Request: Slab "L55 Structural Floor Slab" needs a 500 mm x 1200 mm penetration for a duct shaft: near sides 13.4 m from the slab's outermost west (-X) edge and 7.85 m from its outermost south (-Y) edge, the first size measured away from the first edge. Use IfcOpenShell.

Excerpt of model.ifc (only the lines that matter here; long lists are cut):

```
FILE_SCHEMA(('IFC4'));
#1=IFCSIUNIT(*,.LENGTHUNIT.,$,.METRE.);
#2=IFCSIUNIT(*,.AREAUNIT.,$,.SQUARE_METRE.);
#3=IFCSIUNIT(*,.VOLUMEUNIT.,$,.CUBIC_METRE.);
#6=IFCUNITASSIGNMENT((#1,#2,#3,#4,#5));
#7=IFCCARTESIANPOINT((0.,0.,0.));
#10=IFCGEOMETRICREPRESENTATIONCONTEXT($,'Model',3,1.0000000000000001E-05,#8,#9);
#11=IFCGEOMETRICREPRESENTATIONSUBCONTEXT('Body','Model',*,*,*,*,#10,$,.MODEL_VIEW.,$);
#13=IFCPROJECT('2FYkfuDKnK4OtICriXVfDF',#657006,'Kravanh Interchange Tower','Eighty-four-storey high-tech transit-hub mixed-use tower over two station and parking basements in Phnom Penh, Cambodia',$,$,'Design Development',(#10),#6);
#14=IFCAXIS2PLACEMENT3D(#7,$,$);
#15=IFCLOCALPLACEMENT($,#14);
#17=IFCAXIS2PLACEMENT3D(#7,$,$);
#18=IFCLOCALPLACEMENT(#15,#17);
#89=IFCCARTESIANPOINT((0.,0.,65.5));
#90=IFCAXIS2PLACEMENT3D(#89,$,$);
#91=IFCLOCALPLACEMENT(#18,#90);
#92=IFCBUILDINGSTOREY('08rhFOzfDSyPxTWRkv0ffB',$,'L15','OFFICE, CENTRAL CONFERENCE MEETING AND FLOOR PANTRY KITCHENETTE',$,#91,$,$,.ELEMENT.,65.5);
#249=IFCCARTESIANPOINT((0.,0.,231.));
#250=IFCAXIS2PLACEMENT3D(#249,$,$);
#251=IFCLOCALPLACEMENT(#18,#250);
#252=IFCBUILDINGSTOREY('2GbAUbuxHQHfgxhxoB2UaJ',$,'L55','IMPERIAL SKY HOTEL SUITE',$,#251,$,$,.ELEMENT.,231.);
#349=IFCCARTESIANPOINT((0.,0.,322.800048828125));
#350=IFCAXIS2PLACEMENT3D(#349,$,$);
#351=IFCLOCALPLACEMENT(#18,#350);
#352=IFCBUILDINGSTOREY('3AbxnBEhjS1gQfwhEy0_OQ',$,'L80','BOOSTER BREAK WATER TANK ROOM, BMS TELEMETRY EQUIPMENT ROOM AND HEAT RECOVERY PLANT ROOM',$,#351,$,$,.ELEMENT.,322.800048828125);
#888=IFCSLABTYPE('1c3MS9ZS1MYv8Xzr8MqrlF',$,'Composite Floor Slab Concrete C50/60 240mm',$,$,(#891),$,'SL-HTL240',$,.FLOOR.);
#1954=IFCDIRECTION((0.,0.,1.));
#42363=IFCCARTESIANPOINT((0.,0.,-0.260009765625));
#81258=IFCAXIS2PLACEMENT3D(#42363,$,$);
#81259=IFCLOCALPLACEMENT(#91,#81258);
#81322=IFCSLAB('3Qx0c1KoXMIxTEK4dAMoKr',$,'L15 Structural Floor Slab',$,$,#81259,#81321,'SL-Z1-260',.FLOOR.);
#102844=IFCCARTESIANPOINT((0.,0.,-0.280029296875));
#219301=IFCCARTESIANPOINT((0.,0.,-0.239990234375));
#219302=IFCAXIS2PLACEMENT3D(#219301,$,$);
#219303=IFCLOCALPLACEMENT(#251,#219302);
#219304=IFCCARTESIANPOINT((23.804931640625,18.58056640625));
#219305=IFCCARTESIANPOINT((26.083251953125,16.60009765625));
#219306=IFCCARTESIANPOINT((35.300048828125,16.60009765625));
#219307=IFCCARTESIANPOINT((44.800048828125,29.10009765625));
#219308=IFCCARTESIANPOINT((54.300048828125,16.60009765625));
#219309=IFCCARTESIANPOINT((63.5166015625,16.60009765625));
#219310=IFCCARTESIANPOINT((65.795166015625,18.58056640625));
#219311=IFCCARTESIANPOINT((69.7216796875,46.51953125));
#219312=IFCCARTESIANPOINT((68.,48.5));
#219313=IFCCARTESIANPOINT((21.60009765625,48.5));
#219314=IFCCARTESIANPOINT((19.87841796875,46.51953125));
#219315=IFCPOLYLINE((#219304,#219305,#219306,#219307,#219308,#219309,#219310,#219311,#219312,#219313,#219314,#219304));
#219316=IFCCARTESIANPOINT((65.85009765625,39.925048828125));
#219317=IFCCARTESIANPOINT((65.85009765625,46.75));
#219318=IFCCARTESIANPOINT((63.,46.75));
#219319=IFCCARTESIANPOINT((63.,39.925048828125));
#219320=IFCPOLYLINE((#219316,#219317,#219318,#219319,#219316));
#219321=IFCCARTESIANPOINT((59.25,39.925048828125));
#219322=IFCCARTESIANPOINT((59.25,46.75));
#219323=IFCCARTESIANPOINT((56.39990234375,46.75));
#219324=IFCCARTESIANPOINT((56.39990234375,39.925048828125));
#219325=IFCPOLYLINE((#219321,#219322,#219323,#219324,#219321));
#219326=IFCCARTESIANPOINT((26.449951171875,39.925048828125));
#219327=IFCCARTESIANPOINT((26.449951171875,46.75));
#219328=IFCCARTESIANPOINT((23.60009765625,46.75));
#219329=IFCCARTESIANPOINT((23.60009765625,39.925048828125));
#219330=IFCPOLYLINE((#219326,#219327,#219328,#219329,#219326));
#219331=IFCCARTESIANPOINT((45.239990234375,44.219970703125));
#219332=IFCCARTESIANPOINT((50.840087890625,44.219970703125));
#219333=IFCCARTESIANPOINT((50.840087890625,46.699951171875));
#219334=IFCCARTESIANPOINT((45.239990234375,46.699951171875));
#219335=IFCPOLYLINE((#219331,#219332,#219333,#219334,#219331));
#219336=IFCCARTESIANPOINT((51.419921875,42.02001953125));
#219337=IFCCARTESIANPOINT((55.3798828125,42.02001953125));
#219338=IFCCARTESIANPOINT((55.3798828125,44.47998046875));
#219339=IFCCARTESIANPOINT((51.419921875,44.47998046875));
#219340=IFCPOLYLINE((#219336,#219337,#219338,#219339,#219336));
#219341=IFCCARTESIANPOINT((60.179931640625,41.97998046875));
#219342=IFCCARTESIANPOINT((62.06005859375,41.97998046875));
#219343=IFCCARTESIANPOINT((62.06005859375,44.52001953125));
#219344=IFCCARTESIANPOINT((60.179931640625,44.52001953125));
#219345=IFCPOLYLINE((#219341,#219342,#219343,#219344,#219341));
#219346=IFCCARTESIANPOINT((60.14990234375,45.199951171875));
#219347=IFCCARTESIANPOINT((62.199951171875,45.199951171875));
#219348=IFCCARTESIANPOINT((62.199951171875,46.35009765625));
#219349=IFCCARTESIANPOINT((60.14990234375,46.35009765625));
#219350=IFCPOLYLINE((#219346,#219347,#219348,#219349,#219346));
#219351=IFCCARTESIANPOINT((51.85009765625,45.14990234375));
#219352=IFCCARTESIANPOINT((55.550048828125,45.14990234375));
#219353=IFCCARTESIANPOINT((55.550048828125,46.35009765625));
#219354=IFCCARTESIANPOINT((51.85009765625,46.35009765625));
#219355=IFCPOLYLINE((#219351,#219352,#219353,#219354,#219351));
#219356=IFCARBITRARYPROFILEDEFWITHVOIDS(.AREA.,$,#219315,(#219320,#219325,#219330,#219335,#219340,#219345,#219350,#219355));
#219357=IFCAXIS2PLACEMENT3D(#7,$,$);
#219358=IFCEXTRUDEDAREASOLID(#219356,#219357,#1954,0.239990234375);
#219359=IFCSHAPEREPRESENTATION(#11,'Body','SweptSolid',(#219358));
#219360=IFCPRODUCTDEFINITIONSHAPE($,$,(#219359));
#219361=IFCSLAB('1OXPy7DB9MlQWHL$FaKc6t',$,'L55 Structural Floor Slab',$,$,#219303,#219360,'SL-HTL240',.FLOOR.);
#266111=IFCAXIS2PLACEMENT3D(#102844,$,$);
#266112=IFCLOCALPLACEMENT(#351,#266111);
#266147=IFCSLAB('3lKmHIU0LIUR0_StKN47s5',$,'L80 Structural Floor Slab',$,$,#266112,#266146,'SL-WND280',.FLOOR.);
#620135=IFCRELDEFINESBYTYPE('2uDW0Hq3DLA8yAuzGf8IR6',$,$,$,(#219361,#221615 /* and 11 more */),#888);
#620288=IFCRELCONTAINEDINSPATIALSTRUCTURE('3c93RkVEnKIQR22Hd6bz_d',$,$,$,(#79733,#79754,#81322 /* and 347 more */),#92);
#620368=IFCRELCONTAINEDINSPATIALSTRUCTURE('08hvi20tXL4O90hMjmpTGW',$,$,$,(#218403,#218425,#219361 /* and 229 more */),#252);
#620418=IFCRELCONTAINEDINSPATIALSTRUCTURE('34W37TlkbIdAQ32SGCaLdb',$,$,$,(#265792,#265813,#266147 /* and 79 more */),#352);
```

```python
import numpy as np
import ifcopenshell
import ifcopenshell.api.feature
import ifcopenshell.api.geometry
import ifcopenshell.api.root
import ifcopenshell.geom
import ifcopenshell.util.placement
import ifcopenshell.util.representation
import ifcopenshell.util.shape
import ifcopenshell.util.unit

model = ifcopenshell.open("model.ifc")
unit_scale = ifcopenshell.util.unit.calculate_unit_scale(model)
settings = ifcopenshell.geom.settings()


def volume(element):
    """Net volume in cubic metres, openings subtracted."""
    shape = ifcopenshell.geom.create_shape(settings, element)
    return ifcopenshell.util.shape.get_volume(shape.geometry)


slab = model.by_guid("1OXPy7DB9MlQWHL$FaKc6t")
before = volume(slab)

# Extent in the slab's own axes, in metres. The edges named are its -X and -Y sides.
slab_shape = ifcopenshell.geom.create_shape(settings, slab)
vertices = ifcopenshell.util.shape.get_vertices(slab_shape.geometry)
x_min, y_min, bottom = vertices.min(axis=0)
top = vertices[:, 2].max()

opening = ifcopenshell.api.root.create_entity(model, ifc_class="IfcOpeningElement", name="Duct shaft opening", predefined_type="OPENING")
context = ifcopenshell.util.representation.get_context(model, "Model", "Body", "MODEL_VIEW")
width, depth = 0.5, 1.2
outline = [(0.0, 0.0), (width, 0.0), (width, depth), (0.0, depth), (0.0, 0.0)]
# Overshoot both faces by 50 mm so the cut is clean.
shape = ifcopenshell.api.geometry.add_slab_representation(
    model, context=context, depth=top - bottom + 0.1, polyline=outline
)
ifcopenshell.api.geometry.assign_representation(model, product=opening, representation=shape)

matrix = ifcopenshell.util.placement.get_local_placement(slab.ObjectPlacement)
matrix[:, 3] = matrix @ np.append(np.array([x_min + 13.4, y_min + 7.85, bottom - 0.05]) / unit_scale, 1.0)
ifcopenshell.api.geometry.edit_object_placement(model, product=opening, matrix=matrix, is_si=False)
ifcopenshell.api.feature.add_feature(model, feature=opening, element=slab)

after = volume(slab)

print(f"slab volume {before:.3f} -> {after:.3f} m3")

model.write("model_edited.ifc")
```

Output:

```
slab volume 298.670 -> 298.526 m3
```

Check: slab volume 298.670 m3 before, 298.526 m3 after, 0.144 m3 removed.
